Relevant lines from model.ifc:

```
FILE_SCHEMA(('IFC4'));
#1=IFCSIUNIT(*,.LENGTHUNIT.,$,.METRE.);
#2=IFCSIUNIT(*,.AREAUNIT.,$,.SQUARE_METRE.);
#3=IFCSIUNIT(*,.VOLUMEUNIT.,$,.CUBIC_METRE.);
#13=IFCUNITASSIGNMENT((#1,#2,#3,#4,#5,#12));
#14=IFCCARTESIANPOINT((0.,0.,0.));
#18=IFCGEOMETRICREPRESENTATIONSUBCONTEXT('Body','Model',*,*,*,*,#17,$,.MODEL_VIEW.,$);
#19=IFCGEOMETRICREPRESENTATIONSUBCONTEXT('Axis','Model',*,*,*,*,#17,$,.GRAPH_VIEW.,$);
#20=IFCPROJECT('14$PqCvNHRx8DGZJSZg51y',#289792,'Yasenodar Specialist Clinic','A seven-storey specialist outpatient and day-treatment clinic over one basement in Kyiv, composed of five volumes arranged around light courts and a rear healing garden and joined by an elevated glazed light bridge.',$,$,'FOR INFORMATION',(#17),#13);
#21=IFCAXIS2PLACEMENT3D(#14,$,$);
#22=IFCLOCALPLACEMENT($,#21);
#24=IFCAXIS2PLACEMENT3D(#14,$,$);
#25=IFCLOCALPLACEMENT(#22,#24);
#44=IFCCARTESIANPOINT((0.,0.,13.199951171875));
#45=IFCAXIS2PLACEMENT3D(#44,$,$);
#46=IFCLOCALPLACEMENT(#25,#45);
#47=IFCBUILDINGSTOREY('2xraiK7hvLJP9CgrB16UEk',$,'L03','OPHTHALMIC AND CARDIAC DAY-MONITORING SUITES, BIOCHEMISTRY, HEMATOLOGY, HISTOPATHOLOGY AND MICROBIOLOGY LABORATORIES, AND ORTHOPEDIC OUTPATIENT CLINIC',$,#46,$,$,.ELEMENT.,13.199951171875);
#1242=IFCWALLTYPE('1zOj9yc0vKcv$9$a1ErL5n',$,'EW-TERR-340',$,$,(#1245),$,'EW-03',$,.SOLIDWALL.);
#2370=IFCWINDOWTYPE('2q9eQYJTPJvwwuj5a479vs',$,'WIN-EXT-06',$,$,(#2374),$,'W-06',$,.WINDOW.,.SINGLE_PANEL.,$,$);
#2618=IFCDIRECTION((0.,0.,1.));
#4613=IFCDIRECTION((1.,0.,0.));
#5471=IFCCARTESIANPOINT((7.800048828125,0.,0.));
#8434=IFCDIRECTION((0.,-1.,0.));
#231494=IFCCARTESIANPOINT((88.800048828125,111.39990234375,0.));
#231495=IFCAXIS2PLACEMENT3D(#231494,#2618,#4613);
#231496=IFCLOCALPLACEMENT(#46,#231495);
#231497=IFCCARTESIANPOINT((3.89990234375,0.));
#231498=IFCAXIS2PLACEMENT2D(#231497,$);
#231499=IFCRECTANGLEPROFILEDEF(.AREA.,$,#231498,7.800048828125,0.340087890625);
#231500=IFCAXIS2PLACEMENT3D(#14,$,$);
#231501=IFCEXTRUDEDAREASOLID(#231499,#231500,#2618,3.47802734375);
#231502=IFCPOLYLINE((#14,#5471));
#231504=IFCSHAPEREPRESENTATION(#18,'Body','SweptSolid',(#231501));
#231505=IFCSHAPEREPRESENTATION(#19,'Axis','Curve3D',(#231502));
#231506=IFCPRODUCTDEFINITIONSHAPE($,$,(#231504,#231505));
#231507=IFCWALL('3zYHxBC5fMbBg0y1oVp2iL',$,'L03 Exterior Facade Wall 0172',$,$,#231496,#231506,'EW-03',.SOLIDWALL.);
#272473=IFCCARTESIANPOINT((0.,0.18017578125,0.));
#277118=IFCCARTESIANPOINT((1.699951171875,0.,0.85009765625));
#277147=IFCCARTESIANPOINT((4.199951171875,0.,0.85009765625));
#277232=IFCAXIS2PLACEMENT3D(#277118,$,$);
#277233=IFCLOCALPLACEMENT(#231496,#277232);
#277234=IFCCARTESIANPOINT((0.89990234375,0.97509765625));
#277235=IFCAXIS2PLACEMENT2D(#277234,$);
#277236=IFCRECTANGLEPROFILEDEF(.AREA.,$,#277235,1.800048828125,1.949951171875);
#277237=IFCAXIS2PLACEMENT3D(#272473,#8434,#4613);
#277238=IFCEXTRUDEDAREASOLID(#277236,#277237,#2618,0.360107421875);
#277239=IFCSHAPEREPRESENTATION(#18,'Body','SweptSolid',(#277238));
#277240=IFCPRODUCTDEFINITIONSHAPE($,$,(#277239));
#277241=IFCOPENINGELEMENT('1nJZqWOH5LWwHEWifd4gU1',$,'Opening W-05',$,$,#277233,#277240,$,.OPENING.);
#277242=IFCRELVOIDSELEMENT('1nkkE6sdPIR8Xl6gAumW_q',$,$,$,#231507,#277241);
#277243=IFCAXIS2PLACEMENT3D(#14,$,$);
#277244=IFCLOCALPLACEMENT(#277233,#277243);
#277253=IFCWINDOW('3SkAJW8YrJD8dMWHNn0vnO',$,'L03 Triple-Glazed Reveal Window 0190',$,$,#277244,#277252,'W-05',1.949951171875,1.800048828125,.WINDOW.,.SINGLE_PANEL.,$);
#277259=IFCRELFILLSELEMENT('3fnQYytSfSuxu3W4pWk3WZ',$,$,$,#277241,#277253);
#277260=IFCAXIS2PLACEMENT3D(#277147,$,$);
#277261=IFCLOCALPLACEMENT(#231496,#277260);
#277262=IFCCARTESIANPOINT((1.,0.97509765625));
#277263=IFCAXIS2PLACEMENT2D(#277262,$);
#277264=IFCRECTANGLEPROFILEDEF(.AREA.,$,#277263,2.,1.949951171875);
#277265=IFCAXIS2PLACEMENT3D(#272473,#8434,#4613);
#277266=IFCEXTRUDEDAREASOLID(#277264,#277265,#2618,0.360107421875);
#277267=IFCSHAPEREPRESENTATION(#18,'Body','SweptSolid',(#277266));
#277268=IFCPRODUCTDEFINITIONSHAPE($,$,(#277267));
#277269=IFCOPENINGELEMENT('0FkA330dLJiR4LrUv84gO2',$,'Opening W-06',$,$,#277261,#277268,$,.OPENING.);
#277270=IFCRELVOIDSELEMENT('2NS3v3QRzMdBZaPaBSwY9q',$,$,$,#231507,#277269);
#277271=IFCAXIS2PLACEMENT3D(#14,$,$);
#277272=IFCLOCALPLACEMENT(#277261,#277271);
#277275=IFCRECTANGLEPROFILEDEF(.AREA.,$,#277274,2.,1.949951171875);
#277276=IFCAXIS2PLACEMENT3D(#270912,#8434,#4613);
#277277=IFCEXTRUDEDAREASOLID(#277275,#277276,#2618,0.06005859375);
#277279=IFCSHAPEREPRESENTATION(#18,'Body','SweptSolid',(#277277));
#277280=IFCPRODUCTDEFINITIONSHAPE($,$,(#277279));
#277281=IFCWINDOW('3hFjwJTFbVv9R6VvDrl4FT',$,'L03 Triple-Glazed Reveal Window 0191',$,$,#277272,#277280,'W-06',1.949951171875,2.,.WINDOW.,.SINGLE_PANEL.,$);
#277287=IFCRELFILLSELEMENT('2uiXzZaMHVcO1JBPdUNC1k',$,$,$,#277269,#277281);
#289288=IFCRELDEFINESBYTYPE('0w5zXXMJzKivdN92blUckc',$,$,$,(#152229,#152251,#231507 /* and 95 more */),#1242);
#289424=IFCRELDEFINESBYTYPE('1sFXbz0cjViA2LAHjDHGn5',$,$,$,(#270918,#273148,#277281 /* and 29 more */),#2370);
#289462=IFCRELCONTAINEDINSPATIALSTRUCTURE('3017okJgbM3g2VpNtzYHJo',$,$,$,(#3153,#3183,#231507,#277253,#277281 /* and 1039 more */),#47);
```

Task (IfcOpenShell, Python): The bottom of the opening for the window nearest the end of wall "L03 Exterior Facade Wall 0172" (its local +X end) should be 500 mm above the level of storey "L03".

```python
import numpy as np
import ifcopenshell
import ifcopenshell.api.geometry
import ifcopenshell.geom
import ifcopenshell.util.element
import ifcopenshell.util.placement
import ifcopenshell.util.shape
import ifcopenshell.util.unit

model = ifcopenshell.open("model.ifc")
unit_scale = ifcopenshell.util.unit.calculate_unit_scale(model)

window = model.by_id(277281)
opening = window.FillsVoids[0].RelatingOpeningElement
storey = ifcopenshell.util.element.get_container(window, ifc_class="IfcBuildingStorey")
level = ifcopenshell.util.placement.get_local_placement(storey.ObjectPlacement)[2, 3]

# The opening's origin need not be at the sill, so measure its lowest point.
shape = ifcopenshell.geom.create_shape(ifcopenshell.geom.settings(), opening)
bottom = ifcopenshell.util.shape.get_shape_bottom_elevation(shape, shape.geometry) / unit_scale
dz = level + 0.5 - bottom

shift = np.array([0.0, 0.0, dz])
# The window is placed relative to its opening, so it follows when the opening moves.
matrix = ifcopenshell.util.placement.get_local_placement(opening.ObjectPlacement)
matrix[:3, 3] += shift
ifcopenshell.api.geometry.edit_object_placement(
    model, product=opening, matrix=matrix, is_si=False, should_transform_children=True
)

print(f"moved by {dz * unit_scale:+.3f} m")

model.write("model-out.ifc")
```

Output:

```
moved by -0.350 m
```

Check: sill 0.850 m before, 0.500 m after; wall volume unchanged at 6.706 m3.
